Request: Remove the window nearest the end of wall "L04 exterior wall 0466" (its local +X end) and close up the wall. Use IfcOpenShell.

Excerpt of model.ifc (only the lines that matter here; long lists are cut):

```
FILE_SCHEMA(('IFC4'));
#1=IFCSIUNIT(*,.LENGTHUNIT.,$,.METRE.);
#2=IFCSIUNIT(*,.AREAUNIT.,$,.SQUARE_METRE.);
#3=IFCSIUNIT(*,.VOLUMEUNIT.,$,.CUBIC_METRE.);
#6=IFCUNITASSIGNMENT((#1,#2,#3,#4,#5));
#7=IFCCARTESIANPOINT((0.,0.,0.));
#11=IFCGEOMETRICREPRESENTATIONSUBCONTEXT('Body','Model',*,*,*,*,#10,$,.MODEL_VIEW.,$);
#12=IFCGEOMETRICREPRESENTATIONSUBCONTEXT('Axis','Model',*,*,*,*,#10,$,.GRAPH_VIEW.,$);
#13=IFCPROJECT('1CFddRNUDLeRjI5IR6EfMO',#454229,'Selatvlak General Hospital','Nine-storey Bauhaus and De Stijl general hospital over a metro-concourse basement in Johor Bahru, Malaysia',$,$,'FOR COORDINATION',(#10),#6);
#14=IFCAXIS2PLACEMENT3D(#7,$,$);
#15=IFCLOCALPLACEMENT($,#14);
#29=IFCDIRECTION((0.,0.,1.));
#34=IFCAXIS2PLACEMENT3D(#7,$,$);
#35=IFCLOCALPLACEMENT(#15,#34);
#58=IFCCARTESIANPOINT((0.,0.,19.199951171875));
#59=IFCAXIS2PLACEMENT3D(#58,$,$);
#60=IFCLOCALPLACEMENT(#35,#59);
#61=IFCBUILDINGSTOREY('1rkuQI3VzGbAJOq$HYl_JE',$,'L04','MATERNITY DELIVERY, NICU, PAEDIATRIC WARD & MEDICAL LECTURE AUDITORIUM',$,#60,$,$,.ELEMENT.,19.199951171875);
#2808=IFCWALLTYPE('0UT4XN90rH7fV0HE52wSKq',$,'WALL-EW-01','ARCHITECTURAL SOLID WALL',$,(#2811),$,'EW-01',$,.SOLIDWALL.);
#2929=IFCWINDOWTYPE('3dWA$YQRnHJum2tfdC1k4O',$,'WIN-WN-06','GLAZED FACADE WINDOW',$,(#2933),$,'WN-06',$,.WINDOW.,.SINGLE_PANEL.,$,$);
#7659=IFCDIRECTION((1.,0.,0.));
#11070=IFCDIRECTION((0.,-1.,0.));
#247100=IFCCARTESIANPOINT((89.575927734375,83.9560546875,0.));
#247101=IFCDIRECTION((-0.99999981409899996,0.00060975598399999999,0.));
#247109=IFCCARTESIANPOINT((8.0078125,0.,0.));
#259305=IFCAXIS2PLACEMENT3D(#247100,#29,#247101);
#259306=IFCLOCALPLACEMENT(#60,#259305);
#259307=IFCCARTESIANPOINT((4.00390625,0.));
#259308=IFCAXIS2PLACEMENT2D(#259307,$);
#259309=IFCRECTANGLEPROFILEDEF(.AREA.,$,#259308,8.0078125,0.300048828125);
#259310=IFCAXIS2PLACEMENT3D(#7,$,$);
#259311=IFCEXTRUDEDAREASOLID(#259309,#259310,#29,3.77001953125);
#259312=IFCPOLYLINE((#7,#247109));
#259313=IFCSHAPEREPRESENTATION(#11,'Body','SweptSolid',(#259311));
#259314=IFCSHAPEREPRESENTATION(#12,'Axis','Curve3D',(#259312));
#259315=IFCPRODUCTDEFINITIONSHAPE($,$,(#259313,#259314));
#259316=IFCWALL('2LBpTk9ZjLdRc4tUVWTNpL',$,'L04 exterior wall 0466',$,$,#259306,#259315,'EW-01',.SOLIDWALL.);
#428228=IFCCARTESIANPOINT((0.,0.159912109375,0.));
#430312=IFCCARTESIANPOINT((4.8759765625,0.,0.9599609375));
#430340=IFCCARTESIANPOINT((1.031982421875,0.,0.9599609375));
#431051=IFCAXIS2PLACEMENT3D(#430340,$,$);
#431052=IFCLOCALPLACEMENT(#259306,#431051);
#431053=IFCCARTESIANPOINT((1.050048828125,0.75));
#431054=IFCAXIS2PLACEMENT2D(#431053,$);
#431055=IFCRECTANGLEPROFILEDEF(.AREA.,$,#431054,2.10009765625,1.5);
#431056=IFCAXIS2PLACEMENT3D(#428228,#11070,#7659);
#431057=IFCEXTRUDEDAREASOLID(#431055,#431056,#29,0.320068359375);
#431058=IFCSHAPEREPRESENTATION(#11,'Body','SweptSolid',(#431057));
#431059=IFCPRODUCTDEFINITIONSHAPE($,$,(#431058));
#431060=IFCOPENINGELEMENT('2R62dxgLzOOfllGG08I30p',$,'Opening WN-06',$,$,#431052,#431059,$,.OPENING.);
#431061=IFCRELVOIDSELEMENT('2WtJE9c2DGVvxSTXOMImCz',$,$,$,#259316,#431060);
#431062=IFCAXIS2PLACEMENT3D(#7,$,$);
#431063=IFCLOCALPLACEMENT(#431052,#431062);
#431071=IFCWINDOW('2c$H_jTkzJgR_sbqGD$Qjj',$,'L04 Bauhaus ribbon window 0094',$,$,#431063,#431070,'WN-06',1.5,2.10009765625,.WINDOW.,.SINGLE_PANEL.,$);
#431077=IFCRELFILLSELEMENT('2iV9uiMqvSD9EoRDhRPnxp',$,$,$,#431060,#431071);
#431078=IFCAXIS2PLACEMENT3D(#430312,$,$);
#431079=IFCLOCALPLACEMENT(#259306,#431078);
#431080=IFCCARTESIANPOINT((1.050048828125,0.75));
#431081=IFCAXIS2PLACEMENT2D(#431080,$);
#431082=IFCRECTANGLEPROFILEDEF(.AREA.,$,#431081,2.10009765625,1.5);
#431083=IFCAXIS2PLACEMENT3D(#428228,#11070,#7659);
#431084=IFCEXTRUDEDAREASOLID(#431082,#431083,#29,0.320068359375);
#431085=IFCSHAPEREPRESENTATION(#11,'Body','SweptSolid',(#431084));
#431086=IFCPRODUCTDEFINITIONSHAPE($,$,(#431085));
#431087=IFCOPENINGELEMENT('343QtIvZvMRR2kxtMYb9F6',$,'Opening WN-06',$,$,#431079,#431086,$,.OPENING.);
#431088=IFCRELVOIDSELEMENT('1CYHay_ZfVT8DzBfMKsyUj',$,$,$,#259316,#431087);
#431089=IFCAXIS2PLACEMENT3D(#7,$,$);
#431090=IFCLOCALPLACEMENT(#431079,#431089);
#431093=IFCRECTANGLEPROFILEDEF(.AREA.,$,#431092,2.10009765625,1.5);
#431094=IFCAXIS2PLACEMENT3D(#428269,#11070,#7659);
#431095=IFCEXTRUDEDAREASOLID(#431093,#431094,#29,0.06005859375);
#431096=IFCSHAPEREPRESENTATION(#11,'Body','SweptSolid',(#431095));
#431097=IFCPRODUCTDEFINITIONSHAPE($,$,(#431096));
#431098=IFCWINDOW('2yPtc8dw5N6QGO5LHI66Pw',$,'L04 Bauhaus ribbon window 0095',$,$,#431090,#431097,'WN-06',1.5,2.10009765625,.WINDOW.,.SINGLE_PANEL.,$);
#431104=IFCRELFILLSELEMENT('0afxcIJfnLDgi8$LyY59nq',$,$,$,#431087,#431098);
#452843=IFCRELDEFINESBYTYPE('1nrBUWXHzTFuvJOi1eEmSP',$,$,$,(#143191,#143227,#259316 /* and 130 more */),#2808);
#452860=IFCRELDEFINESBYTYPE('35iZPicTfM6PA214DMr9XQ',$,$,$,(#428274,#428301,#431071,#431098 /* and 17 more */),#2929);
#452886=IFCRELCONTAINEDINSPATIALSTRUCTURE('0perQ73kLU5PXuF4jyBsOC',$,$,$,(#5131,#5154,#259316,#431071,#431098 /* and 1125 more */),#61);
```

```python
import ifcopenshell
import ifcopenshell.api.feature
import ifcopenshell.api.root
import ifcopenshell.geom
import ifcopenshell.util.shape

model = ifcopenshell.open("model.ifc")
settings = ifcopenshell.geom.settings()


def volume(element):
    """Net volume in cubic metres, openings subtracted."""
    shape = ifcopenshell.geom.create_shape(settings, element)
    return ifcopenshell.util.shape.get_volume(shape.geometry)


window = model.by_guid("2yPtc8dw5N6QGO5LHI66Pw")
opening = window.FillsVoids[0].RelatingOpeningElement
wall = opening.VoidsElements[0].RelatingBuildingElement
before = volume(wall)

ifcopenshell.api.root.remove_product(model, product=window)
ifcopenshell.api.feature.remove_feature(model, feature=opening)

after = volume(wall)

print(f"wall volume {before:.3f} -> {after:.3f} m3")

model.write("model-out.ifc")
```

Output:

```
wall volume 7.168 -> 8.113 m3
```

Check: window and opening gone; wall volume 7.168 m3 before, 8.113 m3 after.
